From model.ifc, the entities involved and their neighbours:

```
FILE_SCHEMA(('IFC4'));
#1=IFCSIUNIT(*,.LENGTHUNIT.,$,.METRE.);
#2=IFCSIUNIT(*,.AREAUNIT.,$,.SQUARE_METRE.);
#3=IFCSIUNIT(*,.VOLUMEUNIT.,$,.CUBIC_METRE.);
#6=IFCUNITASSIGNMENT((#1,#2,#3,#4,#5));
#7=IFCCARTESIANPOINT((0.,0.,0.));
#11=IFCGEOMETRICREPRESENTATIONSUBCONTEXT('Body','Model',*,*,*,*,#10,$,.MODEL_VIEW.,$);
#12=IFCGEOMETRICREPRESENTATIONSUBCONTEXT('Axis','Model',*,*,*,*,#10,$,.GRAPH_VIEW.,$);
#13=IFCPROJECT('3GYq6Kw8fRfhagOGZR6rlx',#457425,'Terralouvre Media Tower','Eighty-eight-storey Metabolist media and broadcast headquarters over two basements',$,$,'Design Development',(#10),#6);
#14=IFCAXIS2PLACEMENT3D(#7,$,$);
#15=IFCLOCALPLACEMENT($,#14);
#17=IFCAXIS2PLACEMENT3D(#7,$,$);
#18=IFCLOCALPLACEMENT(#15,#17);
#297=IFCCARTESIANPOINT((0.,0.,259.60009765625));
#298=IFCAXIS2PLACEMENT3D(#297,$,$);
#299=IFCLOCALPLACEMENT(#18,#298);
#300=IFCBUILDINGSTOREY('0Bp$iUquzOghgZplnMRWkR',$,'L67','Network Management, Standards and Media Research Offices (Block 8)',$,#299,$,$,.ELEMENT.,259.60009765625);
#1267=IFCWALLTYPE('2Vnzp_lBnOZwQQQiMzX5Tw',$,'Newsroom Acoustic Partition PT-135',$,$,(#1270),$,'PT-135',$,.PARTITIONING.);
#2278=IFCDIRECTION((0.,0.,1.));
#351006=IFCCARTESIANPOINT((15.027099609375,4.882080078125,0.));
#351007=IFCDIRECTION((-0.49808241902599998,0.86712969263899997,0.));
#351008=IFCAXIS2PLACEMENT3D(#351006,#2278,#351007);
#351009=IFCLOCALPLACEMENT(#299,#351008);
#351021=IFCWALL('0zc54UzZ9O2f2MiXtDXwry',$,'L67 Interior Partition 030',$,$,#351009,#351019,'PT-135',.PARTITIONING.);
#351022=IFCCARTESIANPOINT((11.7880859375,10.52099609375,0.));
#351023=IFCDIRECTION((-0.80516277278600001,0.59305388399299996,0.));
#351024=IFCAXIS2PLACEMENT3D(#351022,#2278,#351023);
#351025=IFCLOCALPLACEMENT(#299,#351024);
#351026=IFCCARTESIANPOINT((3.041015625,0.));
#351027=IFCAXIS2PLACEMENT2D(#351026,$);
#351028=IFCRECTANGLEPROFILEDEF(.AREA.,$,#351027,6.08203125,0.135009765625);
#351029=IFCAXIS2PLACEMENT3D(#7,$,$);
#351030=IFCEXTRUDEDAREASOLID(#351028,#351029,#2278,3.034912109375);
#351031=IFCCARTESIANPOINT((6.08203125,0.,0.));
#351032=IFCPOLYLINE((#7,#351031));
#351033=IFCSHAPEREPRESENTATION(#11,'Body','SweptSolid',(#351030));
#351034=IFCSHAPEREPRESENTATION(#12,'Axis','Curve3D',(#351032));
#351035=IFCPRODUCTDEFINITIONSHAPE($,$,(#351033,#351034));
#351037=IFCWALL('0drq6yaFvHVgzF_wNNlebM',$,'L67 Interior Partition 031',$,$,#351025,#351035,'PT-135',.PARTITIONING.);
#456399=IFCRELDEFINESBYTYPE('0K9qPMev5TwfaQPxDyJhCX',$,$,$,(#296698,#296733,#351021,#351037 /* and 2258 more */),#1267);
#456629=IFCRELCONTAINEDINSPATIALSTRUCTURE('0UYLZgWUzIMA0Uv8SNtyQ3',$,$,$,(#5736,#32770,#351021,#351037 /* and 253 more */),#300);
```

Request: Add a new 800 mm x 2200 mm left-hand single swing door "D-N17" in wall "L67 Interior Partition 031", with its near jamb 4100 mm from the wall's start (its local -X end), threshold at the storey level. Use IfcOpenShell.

```python
import numpy as np
import ifcopenshell
import ifcopenshell.api.feature
import ifcopenshell.api.geometry
import ifcopenshell.api.root
import ifcopenshell.api.spatial
import ifcopenshell.geom
import ifcopenshell.util.element
import ifcopenshell.util.placement
import ifcopenshell.util.representation
import ifcopenshell.util.shape
import ifcopenshell.util.unit

model = ifcopenshell.open("model.ifc")
unit_scale = ifcopenshell.util.unit.calculate_unit_scale(model)
settings = ifcopenshell.geom.settings()


def volume(element):
    """Net volume in cubic metres, openings subtracted."""
    shape = ifcopenshell.geom.create_shape(settings, element)
    return ifcopenshell.util.shape.get_volume(shape.geometry)


wall = model.by_id(351037)
storey = ifcopenshell.util.element.get_container(wall, ifc_class="IfcBuildingStorey")
context = ifcopenshell.util.representation.get_context(model, "Model", "Body", "MODEL_VIEW")
before = volume(wall)

width, height, from_end, sill = 0.8, 2.2, 4.1, 0.0  # metres

# The wall runs along its own X axis, and the end named is its -X end.
wall_shape = ifcopenshell.geom.create_shape(settings, wall)
x, y, z = ifcopenshell.util.shape.get_vertices(wall_shape.geometry).T
start = x.min() + from_end
face, thickness = float(y.min()), float(y.max() - y.min())
wall_matrix = ifcopenshell.util.placement.get_local_placement(wall.ObjectPlacement)
level = ifcopenshell.util.placement.get_local_placement(storey.ObjectPlacement)[2, 3]


def in_wall(x, y):
    """Placement at x, y metres in the wall's axes, at sill height."""
    matrix = wall_matrix.copy()
    matrix[:, 3] = wall_matrix @ np.array([x / unit_scale, y / unit_scale, 0.0, 1.0])
    matrix[2, 3] = level + sill / unit_scale
    return matrix


# Opening: a box that overshoots both wall faces by 50 mm.
opening = ifcopenshell.api.root.create_entity(model, ifc_class="IfcOpeningElement", predefined_type="OPENING")
box = ifcopenshell.api.geometry.add_wall_representation(
    model, context=context, length=width, height=height, thickness=thickness + 0.1
)
ifcopenshell.api.geometry.assign_representation(model, product=opening, representation=box)
ifcopenshell.api.geometry.edit_object_placement(model, product=opening, matrix=in_wall(start, face - 0.05), is_si=False)
ifcopenshell.api.feature.add_feature(model, feature=opening, element=wall)

door = ifcopenshell.api.root.create_entity(model, ifc_class="IfcDoor", name="D-N17", predefined_type="DOOR")
door.OverallWidth, door.OverallHeight = width / unit_scale, height / unit_scale
door.OperationType = "SINGLE_SWING_LEFT"
body = ifcopenshell.api.geometry.add_door_representation(
    model,
    context=context,
    overall_width=door.OverallWidth,
    overall_height=door.OverallHeight,
    operation_type="SINGLE_SWING_LEFT",
    lining_properties={"LiningDepth": thickness / unit_scale, "ThresholdDepth": thickness / unit_scale},
)
ifcopenshell.api.geometry.assign_representation(model, product=door, representation=body)
ifcopenshell.api.spatial.assign_container(model, products=[door], relating_structure=storey)
ifcopenshell.api.feature.add_filling(model, opening=opening, element=door)

# The lining spans the wall, so the door starts at the wall face.
ifcopenshell.api.geometry.edit_object_placement(model, product=door, matrix=in_wall(start, face), is_si=False)

after = volume(wall)

print(f"wall volume {before:.3f} -> {after:.3f} m3")

model.write("model_updated.ifc")
```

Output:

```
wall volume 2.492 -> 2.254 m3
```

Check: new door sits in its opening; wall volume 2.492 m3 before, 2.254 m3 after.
